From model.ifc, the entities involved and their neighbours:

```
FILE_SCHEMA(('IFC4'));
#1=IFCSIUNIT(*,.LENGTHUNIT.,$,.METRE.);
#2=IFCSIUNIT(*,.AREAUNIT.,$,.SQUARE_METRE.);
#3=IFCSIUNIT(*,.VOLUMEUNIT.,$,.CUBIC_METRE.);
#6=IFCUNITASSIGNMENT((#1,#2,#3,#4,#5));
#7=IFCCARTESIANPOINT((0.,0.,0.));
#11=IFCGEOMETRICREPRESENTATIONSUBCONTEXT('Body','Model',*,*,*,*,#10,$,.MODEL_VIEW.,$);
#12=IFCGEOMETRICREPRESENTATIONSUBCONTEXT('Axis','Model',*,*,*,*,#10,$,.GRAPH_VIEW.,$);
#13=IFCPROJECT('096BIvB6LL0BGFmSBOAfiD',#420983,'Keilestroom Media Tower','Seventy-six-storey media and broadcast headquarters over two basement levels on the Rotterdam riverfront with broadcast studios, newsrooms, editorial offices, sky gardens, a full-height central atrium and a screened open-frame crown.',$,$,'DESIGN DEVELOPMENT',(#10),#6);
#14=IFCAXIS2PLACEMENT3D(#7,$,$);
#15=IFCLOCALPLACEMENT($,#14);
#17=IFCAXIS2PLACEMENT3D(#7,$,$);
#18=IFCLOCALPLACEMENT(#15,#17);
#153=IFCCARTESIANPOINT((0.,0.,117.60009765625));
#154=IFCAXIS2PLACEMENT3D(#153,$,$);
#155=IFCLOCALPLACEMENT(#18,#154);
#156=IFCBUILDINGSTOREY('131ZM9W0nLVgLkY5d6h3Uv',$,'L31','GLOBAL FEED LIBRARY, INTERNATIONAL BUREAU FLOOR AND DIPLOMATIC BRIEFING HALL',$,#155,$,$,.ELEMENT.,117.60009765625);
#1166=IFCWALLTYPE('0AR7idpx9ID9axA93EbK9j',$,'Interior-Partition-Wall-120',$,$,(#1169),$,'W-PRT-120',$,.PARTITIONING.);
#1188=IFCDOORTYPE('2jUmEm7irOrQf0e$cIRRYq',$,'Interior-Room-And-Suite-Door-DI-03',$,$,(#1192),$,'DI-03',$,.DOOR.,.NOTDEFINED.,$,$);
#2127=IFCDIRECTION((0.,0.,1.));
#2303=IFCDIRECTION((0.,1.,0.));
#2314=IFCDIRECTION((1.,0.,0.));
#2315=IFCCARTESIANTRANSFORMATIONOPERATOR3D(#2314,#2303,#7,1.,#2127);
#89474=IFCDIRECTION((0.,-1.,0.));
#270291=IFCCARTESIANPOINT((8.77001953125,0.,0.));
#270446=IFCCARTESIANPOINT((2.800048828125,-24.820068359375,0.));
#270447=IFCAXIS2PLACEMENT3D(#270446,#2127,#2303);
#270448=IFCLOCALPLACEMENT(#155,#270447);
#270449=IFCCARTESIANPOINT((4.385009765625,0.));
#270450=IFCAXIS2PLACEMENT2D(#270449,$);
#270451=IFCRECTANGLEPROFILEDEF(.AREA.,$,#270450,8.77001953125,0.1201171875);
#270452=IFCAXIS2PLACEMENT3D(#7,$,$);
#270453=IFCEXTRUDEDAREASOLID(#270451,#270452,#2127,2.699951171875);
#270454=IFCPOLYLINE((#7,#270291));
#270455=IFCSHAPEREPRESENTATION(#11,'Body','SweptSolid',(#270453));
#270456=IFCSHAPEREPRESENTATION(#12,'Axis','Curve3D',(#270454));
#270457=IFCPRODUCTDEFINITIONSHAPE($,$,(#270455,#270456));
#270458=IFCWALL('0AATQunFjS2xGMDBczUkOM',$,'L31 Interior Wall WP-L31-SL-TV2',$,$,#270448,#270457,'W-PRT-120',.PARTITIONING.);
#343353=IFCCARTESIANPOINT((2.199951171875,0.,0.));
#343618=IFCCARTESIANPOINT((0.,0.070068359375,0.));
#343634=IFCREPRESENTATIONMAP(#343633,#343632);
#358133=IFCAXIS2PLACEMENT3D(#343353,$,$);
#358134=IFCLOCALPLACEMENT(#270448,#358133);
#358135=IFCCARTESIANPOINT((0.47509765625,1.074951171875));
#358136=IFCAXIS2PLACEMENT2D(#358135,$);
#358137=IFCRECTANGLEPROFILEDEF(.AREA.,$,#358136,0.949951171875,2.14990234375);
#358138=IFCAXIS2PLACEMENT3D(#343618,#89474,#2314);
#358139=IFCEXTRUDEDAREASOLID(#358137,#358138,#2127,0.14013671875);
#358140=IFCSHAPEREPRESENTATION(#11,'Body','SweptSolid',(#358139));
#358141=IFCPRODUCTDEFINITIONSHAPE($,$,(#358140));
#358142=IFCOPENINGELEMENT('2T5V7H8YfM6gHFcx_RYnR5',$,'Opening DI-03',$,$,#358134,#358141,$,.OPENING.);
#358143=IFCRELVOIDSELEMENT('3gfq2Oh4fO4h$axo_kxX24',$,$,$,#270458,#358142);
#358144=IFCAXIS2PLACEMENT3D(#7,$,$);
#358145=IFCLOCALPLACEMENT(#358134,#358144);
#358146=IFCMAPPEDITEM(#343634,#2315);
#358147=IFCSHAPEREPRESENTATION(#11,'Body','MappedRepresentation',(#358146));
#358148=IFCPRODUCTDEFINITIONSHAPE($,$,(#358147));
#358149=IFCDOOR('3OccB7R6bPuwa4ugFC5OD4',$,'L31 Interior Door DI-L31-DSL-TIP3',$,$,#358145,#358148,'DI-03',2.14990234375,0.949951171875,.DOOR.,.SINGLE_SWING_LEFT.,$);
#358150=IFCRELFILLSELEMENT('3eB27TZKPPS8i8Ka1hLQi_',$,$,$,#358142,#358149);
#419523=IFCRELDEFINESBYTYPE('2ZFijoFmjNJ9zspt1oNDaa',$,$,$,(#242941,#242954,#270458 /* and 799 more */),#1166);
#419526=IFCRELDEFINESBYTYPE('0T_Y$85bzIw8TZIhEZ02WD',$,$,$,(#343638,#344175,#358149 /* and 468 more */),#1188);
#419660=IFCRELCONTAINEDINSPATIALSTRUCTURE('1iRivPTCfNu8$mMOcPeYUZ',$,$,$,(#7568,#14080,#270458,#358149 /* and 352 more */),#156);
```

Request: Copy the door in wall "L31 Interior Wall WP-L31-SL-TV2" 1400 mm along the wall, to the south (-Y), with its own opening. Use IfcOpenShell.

```python
import ifcopenshell
import ifcopenshell.api.feature
import ifcopenshell.api.geometry
import ifcopenshell.api.root
import ifcopenshell.geom
import ifcopenshell.util.element
import ifcopenshell.util.placement
import ifcopenshell.util.shape
import ifcopenshell.util.unit

model = ifcopenshell.open("model.ifc")
unit_scale = ifcopenshell.util.unit.calculate_unit_scale(model)
settings = ifcopenshell.geom.settings()


def volume(element):
    """Net volume in cubic metres, openings subtracted."""
    shape = ifcopenshell.geom.create_shape(settings, element)
    return ifcopenshell.util.shape.get_volume(shape.geometry)


door = model.by_guid("3OccB7R6bPuwa4ugFC5OD4")
opening = door.FillsVoids[0].RelatingOpeningElement
wall = opening.VoidsElements[0].RelatingBuildingElement
before = volume(wall)
shift = ifcopenshell.util.placement.get_local_placement(wall.ObjectPlacement)[:3, 0] * -1.4 / unit_scale

# copy_class copies the void relationship, type, container and properties, but no geometry.
new_opening = ifcopenshell.api.root.copy_class(model, product=opening)
new_opening.Representation = ifcopenshell.util.element.copy_deep(
    model, opening.Representation, exclude=["IfcGeometricRepresentationContext", "IfcRepresentationMap"]
)
new_door = ifcopenshell.api.root.copy_class(model, product=door)
new_door.Representation = ifcopenshell.util.element.copy_deep(
    model, door.Representation, exclude=["IfcGeometricRepresentationContext", "IfcRepresentationMap"]
)
new_door.Tag = None
ifcopenshell.api.feature.add_filling(model, opening=new_opening, element=new_door)

for old, new in ((opening, new_opening), (door, new_door)):
    matrix = ifcopenshell.util.placement.get_local_placement(old.ObjectPlacement)
    matrix[:3, 3] += shift
    ifcopenshell.api.geometry.edit_object_placement(model, product=new, matrix=matrix, is_si=False)

after = volume(wall)

print(f"wall volume {before:.3f} -> {after:.3f} m3")

model.write("model_rev.ifc")
```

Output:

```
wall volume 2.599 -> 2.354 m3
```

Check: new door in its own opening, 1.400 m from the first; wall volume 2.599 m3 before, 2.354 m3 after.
